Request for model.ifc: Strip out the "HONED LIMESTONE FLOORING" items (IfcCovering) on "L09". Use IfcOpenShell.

First a look at what the model holds.

```python
import ifcopenshell
import ifcopenshell.util.element

model = ifcopenshell.open("model.ifc")
print(model.schema)
storey = next(s for s in model.by_type("IfcBuildingStorey") if s.Name == "L09")
coverings = [e for e in ifcopenshell.util.element.get_decomposition(storey) if e.is_a("IfcCovering")]
seen = {}
for e in coverings:
    element_type = ifcopenshell.util.element.get_type(e)
    name = element_type.Name if element_type not in (None, e) else None
    seen[name] = seen.get(name, 0) + 1
for name, count in sorted(seen.items(), key=str):
    print(count, "x", name)
```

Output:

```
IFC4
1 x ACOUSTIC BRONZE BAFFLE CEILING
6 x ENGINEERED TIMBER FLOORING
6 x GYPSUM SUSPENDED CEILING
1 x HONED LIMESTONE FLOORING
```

```python
import ifcopenshell
import ifcopenshell.api.root
import ifcopenshell.util.element

model = ifcopenshell.open("model.ifc")

storey = next(s for s in model.by_type("IfcBuildingStorey") if s.Name == "L09")
coverings = [e for e in ifcopenshell.util.element.get_decomposition(storey) if e.is_a("IfcCovering")]
targets = [e for e in coverings if (t := ifcopenshell.util.element.get_type(e)) not in (None, e) and t.Name == "HONED LIMESTONE FLOORING"]

for e in targets:
    ifcopenshell.api.root.remove_product(model, product=e)
print(len(targets), "removed")

model.write("model_edited.ifc")
```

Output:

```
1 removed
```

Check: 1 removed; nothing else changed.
